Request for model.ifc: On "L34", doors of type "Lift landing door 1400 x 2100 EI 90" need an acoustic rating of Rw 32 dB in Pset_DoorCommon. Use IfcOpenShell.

First a look at what the model holds.

```python
import ifcopenshell
import ifcopenshell.util.element

model = ifcopenshell.open("model.ifc")
print(model.schema)
storey = next(s for s in model.by_type("IfcBuildingStorey") if s.Name == "L34")
doors = [e for e in ifcopenshell.util.element.get_decomposition(storey) if e.is_a("IfcDoor")]
seen = {}
for e in doors:
    element_type = ifcopenshell.util.element.get_type(e)
    key = (element_type.Name if element_type != e and element_type else None, ifcopenshell.util.element.get_pset(e, "Pset_DoorCommon", "AcousticRating"))
    seen[key] = seen.get(key, 0) + 1
for (name, value), count in sorted(seen.items(), key=str):
    print(count, "x", name, "|", value)
```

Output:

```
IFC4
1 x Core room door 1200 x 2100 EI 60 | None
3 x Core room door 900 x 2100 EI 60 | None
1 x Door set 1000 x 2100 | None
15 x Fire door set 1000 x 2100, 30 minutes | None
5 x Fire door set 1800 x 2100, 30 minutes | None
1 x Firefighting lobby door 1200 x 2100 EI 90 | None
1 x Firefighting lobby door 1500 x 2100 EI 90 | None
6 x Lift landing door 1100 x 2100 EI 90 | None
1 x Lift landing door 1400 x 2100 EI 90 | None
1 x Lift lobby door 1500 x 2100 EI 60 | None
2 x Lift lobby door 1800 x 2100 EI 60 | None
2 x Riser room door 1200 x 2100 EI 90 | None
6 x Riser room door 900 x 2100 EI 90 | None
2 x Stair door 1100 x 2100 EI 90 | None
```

```python
import ifcopenshell
import ifcopenshell.api.pset
import ifcopenshell.util.element

model = ifcopenshell.open("model.ifc")

storey = next(s for s in model.by_type("IfcBuildingStorey") if s.Name == "L34")
doors = [e for e in ifcopenshell.util.element.get_decomposition(storey) if e.is_a("IfcDoor")]

count = 0
for e in doors:
    element_type = ifcopenshell.util.element.get_type(e)
    if element_type in (None, e) or element_type.Name != "Lift landing door 1400 x 2100 EI 90":
        continue
    # add_pset returns the element's existing set when there is one.
    pset = ifcopenshell.api.pset.add_pset(model, product=e, name="Pset_DoorCommon")
    ifcopenshell.api.pset.edit_pset(model, pset=pset, properties={"AcousticRating": "Rw 32 dB"})
    count += 1

print(count, "doors updated")

model.write("model_edited.ifc")
```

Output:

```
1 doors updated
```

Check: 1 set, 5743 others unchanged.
